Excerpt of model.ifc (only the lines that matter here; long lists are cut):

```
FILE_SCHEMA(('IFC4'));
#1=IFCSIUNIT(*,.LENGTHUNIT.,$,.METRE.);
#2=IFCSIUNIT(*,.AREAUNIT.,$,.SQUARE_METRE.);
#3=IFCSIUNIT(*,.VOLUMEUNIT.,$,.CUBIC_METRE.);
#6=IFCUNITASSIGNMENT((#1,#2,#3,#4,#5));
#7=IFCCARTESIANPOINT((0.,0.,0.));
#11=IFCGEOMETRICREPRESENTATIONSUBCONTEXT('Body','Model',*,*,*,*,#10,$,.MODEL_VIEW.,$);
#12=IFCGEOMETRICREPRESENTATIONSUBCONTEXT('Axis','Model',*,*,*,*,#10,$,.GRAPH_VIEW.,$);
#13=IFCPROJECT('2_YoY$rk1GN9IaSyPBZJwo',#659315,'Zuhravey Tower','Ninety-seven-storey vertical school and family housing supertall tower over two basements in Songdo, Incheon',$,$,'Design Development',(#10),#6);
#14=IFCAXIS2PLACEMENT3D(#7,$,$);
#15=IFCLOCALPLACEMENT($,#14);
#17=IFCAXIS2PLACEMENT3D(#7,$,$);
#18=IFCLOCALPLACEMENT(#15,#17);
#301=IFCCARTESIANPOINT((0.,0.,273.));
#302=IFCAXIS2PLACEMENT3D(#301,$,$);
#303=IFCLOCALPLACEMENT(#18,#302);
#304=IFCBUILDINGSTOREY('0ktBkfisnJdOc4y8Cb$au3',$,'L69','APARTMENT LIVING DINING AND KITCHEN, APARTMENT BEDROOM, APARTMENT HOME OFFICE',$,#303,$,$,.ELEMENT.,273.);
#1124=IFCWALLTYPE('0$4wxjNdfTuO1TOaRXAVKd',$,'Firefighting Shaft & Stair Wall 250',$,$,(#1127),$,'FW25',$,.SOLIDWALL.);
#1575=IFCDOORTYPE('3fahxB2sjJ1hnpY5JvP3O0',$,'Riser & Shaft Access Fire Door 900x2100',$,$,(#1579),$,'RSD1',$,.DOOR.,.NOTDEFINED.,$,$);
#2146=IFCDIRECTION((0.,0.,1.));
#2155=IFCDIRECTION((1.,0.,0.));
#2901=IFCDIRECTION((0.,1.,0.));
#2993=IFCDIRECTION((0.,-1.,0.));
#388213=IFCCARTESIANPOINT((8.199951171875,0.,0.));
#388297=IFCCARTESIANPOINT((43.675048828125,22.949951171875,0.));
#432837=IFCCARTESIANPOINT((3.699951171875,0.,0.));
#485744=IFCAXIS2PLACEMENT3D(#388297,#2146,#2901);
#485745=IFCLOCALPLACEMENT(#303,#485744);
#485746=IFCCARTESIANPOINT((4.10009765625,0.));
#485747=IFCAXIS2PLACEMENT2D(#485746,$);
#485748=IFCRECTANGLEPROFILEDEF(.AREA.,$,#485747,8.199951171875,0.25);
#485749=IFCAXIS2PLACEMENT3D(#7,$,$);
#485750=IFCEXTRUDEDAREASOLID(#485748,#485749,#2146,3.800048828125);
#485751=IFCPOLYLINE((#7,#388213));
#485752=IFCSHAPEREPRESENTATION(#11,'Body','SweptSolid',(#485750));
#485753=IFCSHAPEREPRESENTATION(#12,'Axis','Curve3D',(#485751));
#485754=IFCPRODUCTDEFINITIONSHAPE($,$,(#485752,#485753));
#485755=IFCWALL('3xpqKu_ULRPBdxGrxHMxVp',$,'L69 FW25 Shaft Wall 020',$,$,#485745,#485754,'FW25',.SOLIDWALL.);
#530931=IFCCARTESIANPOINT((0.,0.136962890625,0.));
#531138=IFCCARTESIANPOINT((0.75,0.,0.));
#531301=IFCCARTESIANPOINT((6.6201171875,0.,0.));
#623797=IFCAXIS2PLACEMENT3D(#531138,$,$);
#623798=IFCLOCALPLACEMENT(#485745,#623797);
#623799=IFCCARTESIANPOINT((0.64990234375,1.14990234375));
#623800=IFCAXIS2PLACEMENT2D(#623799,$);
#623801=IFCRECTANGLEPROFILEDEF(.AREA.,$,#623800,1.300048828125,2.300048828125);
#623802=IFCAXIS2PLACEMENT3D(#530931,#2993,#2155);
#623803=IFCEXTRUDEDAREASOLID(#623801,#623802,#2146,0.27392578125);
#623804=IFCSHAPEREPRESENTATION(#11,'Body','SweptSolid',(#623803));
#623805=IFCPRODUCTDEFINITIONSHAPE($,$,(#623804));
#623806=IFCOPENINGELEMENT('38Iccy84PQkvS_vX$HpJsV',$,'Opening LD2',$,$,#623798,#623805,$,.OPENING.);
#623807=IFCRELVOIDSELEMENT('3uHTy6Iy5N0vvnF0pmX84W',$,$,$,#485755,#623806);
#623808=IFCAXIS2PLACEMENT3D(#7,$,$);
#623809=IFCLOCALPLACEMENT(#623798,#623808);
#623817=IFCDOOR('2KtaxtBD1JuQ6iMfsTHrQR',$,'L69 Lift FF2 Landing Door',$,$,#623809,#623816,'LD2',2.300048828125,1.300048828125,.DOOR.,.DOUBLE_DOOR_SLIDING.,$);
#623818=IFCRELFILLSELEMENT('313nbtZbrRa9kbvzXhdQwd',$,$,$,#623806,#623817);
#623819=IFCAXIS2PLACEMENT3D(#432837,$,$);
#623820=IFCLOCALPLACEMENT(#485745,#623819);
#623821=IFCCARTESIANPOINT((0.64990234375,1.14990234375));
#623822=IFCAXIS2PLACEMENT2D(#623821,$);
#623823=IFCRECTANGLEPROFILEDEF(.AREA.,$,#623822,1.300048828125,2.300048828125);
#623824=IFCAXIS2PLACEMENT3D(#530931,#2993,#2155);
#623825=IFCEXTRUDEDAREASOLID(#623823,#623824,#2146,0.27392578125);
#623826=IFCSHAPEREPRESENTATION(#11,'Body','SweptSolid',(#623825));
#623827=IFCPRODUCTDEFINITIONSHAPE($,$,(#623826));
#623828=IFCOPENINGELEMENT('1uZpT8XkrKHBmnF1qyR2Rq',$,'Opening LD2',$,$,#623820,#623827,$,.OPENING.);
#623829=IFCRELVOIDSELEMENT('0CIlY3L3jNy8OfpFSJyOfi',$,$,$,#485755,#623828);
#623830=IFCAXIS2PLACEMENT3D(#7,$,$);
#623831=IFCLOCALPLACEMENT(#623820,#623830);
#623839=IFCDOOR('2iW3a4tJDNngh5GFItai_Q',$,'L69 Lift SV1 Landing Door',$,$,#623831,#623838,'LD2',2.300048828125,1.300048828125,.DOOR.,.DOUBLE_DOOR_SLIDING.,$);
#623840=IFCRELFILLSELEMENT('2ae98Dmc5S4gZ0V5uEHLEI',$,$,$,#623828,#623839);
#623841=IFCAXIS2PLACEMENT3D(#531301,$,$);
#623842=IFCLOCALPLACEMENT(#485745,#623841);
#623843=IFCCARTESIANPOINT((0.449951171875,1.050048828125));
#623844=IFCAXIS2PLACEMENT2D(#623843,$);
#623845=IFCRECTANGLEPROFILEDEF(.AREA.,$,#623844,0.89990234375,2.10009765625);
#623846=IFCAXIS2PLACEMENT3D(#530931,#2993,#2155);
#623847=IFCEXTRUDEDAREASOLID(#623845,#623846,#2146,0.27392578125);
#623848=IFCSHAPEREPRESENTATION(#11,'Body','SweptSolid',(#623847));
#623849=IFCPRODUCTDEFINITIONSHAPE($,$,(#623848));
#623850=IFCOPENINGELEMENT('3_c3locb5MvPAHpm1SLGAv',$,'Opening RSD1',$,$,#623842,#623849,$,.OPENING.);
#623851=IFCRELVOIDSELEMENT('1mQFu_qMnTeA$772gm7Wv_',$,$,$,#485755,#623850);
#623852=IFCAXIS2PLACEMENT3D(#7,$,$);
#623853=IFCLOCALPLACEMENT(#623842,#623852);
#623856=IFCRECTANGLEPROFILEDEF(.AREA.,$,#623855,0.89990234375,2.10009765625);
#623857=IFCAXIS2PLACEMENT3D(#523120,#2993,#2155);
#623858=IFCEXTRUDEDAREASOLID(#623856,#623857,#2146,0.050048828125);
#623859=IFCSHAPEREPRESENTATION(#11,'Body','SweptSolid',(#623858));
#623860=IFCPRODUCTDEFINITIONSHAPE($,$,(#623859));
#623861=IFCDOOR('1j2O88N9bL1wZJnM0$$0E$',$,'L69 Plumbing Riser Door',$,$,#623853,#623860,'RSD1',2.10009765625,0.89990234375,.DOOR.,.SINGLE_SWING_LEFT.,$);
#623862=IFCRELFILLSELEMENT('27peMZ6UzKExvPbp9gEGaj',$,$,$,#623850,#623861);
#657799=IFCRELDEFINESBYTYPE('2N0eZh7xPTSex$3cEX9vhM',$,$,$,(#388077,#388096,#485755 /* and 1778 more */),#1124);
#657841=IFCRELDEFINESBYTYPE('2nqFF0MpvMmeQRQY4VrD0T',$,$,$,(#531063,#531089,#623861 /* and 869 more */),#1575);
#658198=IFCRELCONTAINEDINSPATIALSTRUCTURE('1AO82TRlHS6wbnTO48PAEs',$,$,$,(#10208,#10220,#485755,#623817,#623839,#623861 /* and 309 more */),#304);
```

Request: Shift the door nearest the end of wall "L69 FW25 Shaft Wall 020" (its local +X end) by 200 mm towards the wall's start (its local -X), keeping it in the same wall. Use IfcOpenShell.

```python
import ifcopenshell
import ifcopenshell.api.geometry
import ifcopenshell.util.placement
import ifcopenshell.util.unit

model = ifcopenshell.open("model.ifc")
unit_scale = ifcopenshell.util.unit.calculate_unit_scale(model)

door = model.by_guid("1j2O88N9bL1wZJnM0$$0E$")
opening = door.FillsVoids[0].RelatingOpeningElement
wall = opening.VoidsElements[0].RelatingBuildingElement

wall_matrix = ifcopenshell.util.placement.get_local_placement(wall.ObjectPlacement)
shift = wall_matrix[:3, 0] * -0.2 / unit_scale
before = ifcopenshell.util.placement.get_local_placement(door.ObjectPlacement)[:3, 3].copy()

# The door is placed relative to its opening, so it follows when the opening moves.
matrix = ifcopenshell.util.placement.get_local_placement(opening.ObjectPlacement)
matrix[:3, 3] += shift
ifcopenshell.api.geometry.edit_object_placement(
    model, product=opening, matrix=matrix, is_si=False, should_transform_children=True
)

after = ifcopenshell.util.placement.get_local_placement(door.ObjectPlacement)[:3, 3]
print("door moved by", (after - before).round(3) + 0.0)

model.write("model-out.ifc")
```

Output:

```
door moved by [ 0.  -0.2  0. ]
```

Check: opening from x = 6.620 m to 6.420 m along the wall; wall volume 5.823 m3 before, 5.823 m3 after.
